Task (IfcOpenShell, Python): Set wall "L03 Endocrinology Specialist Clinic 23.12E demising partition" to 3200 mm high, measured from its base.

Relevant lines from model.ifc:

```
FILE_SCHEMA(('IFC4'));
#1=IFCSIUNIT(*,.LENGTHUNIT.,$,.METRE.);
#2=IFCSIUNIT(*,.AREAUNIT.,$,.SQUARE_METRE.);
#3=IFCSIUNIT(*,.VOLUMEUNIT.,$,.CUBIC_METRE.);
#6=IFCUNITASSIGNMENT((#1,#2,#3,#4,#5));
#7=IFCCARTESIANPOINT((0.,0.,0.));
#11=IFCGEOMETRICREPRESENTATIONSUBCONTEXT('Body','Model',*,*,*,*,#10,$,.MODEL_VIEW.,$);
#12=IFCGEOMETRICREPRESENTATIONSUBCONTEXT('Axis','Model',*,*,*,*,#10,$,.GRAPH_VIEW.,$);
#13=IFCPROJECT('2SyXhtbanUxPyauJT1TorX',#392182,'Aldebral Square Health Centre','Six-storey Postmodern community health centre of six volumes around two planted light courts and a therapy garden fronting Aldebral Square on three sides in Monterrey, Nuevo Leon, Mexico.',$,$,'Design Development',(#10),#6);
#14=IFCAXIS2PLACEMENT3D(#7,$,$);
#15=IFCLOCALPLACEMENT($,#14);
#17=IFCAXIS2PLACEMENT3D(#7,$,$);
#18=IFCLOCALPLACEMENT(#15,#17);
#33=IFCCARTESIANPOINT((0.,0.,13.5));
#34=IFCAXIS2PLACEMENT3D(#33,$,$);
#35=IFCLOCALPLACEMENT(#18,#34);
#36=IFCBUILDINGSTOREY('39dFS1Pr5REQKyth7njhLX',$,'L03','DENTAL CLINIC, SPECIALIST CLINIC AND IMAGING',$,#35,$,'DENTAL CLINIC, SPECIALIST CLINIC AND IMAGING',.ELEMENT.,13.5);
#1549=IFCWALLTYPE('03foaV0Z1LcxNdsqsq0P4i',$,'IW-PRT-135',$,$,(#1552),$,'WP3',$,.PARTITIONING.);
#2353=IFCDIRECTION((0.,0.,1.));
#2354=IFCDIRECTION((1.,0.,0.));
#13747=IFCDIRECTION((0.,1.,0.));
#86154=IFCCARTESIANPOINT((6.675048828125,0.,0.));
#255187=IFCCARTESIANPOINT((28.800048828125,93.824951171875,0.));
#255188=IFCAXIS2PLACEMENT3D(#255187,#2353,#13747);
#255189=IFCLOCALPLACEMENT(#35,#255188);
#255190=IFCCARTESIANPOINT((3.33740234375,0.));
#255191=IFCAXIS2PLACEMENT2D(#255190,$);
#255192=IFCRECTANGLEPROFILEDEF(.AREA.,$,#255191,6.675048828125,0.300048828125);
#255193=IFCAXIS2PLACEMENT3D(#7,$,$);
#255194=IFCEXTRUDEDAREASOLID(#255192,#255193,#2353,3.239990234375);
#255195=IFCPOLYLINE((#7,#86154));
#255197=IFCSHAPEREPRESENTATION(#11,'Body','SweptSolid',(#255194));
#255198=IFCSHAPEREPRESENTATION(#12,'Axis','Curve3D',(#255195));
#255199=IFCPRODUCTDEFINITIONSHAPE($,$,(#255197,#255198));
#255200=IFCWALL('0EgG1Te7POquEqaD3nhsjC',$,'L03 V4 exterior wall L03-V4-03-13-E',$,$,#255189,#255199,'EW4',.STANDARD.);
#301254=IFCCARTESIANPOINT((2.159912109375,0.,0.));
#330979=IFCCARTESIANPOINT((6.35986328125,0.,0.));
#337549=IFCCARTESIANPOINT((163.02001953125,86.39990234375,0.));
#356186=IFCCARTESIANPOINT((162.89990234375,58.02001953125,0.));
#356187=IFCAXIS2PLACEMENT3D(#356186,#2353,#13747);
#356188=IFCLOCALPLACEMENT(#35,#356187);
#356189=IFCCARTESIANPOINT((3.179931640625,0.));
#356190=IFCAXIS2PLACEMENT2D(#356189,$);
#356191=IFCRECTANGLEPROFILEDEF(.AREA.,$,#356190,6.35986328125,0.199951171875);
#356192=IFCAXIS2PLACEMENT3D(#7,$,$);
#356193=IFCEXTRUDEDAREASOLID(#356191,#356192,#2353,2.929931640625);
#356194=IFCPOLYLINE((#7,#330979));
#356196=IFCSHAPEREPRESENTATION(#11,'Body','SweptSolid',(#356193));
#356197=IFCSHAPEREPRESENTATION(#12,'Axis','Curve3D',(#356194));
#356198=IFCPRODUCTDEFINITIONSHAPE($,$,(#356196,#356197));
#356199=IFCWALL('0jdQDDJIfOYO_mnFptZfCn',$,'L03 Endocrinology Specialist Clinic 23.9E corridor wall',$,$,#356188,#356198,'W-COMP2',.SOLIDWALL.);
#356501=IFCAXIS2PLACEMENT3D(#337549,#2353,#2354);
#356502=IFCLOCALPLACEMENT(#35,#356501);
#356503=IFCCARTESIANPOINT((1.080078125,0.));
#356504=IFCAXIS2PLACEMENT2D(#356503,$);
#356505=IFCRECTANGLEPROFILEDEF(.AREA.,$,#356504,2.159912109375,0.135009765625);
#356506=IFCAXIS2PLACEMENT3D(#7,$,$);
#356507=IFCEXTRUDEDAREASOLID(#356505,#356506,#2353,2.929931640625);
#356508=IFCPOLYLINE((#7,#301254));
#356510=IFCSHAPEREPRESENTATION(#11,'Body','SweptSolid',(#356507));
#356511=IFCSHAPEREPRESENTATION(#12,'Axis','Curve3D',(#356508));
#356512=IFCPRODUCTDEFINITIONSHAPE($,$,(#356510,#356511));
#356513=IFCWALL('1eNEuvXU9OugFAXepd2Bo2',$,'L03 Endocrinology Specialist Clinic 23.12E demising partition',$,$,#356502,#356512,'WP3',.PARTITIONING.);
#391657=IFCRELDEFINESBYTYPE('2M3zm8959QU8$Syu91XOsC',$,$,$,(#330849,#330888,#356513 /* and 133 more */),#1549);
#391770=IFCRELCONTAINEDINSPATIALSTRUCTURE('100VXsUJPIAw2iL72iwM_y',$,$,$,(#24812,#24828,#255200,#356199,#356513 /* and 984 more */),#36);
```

```python
import ifcopenshell
import ifcopenshell.geom
import ifcopenshell.util.representation
import ifcopenshell.util.shape
import ifcopenshell.util.unit

model = ifcopenshell.open("model.ifc")
unit_scale = ifcopenshell.util.unit.calculate_unit_scale(model)
settings = ifcopenshell.geom.settings()


def volume(element):
    """Net volume in cubic metres, openings subtracted."""
    shape = ifcopenshell.geom.create_shape(settings, element)
    return ifcopenshell.util.shape.get_volume(shape.geometry)


wall = model.by_id(356513)
before = volume(wall)

body = ifcopenshell.util.representation.get_representation(wall, "Model", "Body")
solid = body.Items[0]
old_height = solid.Depth
solid.Depth = 3.2 / unit_scale
after = volume(wall)

print(f"height {old_height:g} -> {solid.Depth:g}, volume {before:.3f} -> {after:.3f} m3")

model.write("model-out.ifc")
```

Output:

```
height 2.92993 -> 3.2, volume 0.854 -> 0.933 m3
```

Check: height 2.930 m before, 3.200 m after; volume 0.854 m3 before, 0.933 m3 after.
